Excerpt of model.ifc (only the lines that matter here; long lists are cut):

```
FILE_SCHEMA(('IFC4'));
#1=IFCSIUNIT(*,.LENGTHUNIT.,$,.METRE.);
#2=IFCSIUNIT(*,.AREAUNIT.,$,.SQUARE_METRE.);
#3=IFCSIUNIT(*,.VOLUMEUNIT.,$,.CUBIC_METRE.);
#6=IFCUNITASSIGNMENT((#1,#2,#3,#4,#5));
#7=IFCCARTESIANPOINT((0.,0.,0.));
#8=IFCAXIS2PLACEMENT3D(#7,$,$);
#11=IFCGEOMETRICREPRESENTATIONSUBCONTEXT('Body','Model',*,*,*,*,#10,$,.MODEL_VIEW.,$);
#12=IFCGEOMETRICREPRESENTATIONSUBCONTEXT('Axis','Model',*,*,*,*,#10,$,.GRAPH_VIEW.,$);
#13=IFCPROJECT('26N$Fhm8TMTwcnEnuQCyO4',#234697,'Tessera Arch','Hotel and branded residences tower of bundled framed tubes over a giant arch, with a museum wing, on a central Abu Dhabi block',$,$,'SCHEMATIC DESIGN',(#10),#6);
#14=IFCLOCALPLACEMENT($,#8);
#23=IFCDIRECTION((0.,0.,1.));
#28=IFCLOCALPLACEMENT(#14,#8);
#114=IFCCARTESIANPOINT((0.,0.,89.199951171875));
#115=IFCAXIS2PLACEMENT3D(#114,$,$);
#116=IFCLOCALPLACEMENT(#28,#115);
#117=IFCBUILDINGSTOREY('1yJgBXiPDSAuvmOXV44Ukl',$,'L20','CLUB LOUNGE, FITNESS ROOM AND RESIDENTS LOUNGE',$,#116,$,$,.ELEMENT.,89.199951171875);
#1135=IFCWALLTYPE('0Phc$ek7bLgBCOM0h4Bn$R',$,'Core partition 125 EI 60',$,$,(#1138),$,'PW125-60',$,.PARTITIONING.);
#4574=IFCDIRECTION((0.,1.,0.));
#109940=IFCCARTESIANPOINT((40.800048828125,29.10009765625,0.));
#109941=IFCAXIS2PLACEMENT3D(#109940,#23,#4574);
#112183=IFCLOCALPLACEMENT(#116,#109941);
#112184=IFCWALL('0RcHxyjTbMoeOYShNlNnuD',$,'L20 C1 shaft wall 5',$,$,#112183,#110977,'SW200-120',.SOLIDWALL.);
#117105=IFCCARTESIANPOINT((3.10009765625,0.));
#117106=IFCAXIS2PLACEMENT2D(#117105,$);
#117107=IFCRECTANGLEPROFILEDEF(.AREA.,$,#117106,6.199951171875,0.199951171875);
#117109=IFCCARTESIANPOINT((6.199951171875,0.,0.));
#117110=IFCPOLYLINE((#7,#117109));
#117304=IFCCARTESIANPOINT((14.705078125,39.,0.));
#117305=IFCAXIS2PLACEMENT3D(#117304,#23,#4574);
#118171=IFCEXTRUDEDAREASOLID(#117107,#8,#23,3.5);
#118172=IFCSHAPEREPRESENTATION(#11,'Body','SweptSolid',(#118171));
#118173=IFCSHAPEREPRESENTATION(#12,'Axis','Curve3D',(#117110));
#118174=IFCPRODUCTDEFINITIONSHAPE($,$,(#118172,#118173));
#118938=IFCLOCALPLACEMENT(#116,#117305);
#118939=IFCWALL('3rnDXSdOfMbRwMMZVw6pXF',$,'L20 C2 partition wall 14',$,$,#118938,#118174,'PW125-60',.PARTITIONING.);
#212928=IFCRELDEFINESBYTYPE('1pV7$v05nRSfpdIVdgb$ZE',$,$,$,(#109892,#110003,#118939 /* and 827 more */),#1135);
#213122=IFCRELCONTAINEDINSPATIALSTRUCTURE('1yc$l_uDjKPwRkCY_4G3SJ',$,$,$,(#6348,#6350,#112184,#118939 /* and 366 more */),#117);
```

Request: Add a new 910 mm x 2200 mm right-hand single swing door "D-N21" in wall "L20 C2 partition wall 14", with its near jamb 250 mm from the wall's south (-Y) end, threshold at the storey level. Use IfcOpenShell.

```python
import numpy as np
import ifcopenshell
import ifcopenshell.api.feature
import ifcopenshell.api.geometry
import ifcopenshell.api.root
import ifcopenshell.api.spatial
import ifcopenshell.geom
import ifcopenshell.util.element
import ifcopenshell.util.placement
import ifcopenshell.util.representation
import ifcopenshell.util.shape
import ifcopenshell.util.unit

model = ifcopenshell.open("model.ifc")
unit_scale = ifcopenshell.util.unit.calculate_unit_scale(model)
settings = ifcopenshell.geom.settings()


def volume(element):
    """Net volume in cubic metres, openings subtracted."""
    shape = ifcopenshell.geom.create_shape(settings, element)
    return ifcopenshell.util.shape.get_volume(shape.geometry)


wall = model.by_guid("3rnDXSdOfMbRwMMZVw6pXF")
storey = ifcopenshell.util.element.get_container(wall, ifc_class="IfcBuildingStorey")
context = ifcopenshell.util.representation.get_context(model, "Model", "Body", "MODEL_VIEW")
before = volume(wall)

width, height, from_end, sill = 0.91, 2.2, 0.25, 0.0  # metres

# The wall runs along its own X axis, and the end named is its -X end.
wall_shape = ifcopenshell.geom.create_shape(settings, wall)
x, y, z = ifcopenshell.util.shape.get_vertices(wall_shape.geometry).T
start = x.min() + from_end
face, thickness = float(y.min()), float(y.max() - y.min())
wall_matrix = ifcopenshell.util.placement.get_local_placement(wall.ObjectPlacement)
level = ifcopenshell.util.placement.get_local_placement(storey.ObjectPlacement)[2, 3]


def in_wall(x, y):
    """Placement at x, y metres in the wall's axes, at sill height."""
    matrix = wall_matrix.copy()
    matrix[:, 3] = wall_matrix @ np.array([x / unit_scale, y / unit_scale, 0.0, 1.0])
    matrix[2, 3] = level + sill / unit_scale
    return matrix


# Opening: a box that overshoots both wall faces by 50 mm.
opening = ifcopenshell.api.root.create_entity(model, ifc_class="IfcOpeningElement", predefined_type="OPENING")
box = ifcopenshell.api.geometry.add_wall_representation(
    model, context=context, length=width, height=height, thickness=thickness + 0.1
)
ifcopenshell.api.geometry.assign_representation(model, product=opening, representation=box)
ifcopenshell.api.geometry.edit_object_placement(model, product=opening, matrix=in_wall(start, face - 0.05), is_si=False)
ifcopenshell.api.feature.add_feature(model, feature=opening, element=wall)

door = ifcopenshell.api.root.create_entity(model, ifc_class="IfcDoor", name="D-N21", predefined_type="DOOR")
door.OverallWidth, door.OverallHeight = width / unit_scale, height / unit_scale
door.OperationType = "SINGLE_SWING_RIGHT"
body = ifcopenshell.api.geometry.add_door_representation(
    model,
    context=context,
    overall_width=door.OverallWidth,
    overall_height=door.OverallHeight,
    operation_type="SINGLE_SWING_RIGHT",
    lining_properties={"LiningDepth": thickness / unit_scale, "ThresholdDepth": thickness / unit_scale},
)
ifcopenshell.api.geometry.assign_representation(model, product=door, representation=body)
ifcopenshell.api.spatial.assign_container(model, products=[door], relating_structure=storey)
ifcopenshell.api.feature.add_filling(model, opening=opening, element=door)

# The lining spans the wall, so the door starts at the wall face.
ifcopenshell.api.geometry.edit_object_placement(model, product=door, matrix=in_wall(start, face), is_si=False)

after = volume(wall)

print(f"wall volume {before:.3f} -> {after:.3f} m3")

model.write("model_edited.ifc")
```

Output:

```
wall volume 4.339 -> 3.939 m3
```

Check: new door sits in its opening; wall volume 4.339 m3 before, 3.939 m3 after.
